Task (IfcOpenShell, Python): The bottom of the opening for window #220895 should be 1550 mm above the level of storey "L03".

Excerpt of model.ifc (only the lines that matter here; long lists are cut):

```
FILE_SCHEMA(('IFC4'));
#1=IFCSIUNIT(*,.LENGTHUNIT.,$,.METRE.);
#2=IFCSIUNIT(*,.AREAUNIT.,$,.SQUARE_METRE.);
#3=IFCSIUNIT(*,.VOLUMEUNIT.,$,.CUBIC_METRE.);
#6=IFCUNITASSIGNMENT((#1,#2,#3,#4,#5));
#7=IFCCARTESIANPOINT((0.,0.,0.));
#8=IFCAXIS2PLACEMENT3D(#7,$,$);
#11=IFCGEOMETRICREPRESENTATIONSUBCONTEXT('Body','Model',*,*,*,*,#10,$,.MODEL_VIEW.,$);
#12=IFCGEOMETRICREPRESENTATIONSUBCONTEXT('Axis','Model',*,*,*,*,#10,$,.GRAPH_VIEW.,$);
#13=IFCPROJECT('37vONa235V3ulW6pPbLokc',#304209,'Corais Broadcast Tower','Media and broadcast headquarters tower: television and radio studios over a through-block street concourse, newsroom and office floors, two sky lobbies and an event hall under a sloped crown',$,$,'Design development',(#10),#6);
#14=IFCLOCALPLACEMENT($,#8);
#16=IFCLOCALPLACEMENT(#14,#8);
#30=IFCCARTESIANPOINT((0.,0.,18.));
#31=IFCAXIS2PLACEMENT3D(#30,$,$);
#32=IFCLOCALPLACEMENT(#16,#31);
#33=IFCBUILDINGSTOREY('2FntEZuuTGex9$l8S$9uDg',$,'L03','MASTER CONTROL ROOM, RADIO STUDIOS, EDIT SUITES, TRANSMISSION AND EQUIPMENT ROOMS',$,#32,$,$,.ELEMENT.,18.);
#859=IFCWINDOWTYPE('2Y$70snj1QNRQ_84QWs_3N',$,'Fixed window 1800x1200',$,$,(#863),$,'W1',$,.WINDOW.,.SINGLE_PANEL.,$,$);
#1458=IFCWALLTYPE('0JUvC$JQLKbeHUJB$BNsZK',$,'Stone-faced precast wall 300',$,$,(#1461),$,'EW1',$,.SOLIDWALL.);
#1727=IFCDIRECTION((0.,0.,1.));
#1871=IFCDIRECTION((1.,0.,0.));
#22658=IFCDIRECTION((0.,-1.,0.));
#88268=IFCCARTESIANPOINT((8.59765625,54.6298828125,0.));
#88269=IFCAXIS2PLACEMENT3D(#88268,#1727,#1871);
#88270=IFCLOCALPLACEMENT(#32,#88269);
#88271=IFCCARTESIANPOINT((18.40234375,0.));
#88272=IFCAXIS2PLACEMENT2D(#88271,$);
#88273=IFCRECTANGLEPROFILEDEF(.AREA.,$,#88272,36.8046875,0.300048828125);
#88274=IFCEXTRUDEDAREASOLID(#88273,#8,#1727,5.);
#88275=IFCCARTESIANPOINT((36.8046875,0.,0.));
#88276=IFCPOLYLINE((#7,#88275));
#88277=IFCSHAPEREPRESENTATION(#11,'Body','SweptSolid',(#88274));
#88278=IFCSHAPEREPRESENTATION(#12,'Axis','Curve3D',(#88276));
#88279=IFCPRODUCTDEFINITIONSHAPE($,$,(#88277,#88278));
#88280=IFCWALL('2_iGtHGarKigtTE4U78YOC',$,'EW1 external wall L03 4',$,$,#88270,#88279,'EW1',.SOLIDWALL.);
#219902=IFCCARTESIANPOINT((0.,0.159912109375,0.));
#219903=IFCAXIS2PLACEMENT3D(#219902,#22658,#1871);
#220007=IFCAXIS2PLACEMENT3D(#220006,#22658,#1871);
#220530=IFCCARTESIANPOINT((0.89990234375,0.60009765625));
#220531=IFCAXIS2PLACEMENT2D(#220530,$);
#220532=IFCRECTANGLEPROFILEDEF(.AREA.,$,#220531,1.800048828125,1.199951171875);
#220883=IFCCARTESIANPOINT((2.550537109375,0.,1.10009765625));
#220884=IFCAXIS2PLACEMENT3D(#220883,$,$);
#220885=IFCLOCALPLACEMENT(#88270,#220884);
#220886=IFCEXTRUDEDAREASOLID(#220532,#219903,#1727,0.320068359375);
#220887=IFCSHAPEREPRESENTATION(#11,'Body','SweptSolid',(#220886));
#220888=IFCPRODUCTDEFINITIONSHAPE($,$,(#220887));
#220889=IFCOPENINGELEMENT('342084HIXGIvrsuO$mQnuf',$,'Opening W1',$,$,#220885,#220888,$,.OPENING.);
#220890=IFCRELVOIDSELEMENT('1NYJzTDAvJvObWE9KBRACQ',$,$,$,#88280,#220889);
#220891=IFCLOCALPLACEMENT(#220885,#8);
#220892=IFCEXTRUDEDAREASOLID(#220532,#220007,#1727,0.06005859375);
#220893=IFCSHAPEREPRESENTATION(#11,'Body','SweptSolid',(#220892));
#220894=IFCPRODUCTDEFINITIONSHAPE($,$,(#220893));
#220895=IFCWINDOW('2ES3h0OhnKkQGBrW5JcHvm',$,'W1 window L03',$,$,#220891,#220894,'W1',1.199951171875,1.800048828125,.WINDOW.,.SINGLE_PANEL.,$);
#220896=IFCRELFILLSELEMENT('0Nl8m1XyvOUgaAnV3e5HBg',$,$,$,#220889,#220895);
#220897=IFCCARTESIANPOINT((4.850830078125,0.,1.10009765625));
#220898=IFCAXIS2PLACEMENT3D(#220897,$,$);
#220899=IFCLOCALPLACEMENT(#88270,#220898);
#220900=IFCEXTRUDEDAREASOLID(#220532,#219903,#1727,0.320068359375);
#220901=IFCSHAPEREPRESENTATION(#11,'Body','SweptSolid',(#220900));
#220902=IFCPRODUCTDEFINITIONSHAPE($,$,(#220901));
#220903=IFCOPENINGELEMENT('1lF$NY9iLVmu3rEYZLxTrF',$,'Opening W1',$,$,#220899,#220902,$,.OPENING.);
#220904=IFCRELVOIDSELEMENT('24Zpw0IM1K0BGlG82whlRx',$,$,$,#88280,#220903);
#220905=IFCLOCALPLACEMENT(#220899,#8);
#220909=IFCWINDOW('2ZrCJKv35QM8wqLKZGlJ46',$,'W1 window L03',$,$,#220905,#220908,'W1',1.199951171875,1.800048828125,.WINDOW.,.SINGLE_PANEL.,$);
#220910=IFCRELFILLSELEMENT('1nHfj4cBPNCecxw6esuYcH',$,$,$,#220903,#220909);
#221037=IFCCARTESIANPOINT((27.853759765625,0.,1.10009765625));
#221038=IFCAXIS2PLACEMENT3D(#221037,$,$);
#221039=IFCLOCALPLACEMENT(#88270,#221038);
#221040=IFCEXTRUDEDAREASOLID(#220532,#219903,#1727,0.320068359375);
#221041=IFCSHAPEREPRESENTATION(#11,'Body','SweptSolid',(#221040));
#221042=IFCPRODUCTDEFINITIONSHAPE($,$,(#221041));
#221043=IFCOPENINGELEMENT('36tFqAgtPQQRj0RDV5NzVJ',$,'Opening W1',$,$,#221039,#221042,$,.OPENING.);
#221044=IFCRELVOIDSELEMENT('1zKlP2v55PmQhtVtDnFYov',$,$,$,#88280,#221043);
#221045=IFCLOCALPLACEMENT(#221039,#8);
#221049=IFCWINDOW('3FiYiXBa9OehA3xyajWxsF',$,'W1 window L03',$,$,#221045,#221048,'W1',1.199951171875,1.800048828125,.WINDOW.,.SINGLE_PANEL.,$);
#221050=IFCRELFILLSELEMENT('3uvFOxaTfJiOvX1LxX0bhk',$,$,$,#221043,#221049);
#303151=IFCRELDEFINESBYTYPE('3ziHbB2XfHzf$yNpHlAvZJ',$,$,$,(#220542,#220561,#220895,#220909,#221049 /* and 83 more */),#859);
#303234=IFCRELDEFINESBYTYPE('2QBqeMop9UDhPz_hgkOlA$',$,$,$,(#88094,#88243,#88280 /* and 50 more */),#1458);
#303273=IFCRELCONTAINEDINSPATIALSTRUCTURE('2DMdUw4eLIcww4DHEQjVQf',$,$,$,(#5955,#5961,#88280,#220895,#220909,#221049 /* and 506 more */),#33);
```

```python
import numpy as np
import ifcopenshell
import ifcopenshell.api.geometry
import ifcopenshell.geom
import ifcopenshell.util.element
import ifcopenshell.util.placement
import ifcopenshell.util.shape
import ifcopenshell.util.unit

model = ifcopenshell.open("model.ifc")
unit_scale = ifcopenshell.util.unit.calculate_unit_scale(model)

window = model.by_guid("2ES3h0OhnKkQGBrW5JcHvm")
opening = window.FillsVoids[0].RelatingOpeningElement
storey = ifcopenshell.util.element.get_container(window, ifc_class="IfcBuildingStorey")
level = ifcopenshell.util.placement.get_local_placement(storey.ObjectPlacement)[2, 3]

# The opening's origin need not be at the sill, so measure its lowest point.
shape = ifcopenshell.geom.create_shape(ifcopenshell.geom.settings(), opening)
bottom = ifcopenshell.util.shape.get_shape_bottom_elevation(shape, shape.geometry) / unit_scale
dz = level + 1.55 / unit_scale - bottom

shift = np.array([0.0, 0.0, dz])
# The window is placed relative to its opening, so it follows when the opening moves.
matrix = ifcopenshell.util.placement.get_local_placement(opening.ObjectPlacement)
matrix[:3, 3] += shift
ifcopenshell.api.geometry.edit_object_placement(
    model, product=opening, matrix=matrix, is_si=False, should_transform_children=True
)

print(f"moved by {dz * unit_scale:+.3f} m")

model.write("model_updated.ifc")
```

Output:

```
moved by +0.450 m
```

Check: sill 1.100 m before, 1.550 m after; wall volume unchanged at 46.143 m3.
